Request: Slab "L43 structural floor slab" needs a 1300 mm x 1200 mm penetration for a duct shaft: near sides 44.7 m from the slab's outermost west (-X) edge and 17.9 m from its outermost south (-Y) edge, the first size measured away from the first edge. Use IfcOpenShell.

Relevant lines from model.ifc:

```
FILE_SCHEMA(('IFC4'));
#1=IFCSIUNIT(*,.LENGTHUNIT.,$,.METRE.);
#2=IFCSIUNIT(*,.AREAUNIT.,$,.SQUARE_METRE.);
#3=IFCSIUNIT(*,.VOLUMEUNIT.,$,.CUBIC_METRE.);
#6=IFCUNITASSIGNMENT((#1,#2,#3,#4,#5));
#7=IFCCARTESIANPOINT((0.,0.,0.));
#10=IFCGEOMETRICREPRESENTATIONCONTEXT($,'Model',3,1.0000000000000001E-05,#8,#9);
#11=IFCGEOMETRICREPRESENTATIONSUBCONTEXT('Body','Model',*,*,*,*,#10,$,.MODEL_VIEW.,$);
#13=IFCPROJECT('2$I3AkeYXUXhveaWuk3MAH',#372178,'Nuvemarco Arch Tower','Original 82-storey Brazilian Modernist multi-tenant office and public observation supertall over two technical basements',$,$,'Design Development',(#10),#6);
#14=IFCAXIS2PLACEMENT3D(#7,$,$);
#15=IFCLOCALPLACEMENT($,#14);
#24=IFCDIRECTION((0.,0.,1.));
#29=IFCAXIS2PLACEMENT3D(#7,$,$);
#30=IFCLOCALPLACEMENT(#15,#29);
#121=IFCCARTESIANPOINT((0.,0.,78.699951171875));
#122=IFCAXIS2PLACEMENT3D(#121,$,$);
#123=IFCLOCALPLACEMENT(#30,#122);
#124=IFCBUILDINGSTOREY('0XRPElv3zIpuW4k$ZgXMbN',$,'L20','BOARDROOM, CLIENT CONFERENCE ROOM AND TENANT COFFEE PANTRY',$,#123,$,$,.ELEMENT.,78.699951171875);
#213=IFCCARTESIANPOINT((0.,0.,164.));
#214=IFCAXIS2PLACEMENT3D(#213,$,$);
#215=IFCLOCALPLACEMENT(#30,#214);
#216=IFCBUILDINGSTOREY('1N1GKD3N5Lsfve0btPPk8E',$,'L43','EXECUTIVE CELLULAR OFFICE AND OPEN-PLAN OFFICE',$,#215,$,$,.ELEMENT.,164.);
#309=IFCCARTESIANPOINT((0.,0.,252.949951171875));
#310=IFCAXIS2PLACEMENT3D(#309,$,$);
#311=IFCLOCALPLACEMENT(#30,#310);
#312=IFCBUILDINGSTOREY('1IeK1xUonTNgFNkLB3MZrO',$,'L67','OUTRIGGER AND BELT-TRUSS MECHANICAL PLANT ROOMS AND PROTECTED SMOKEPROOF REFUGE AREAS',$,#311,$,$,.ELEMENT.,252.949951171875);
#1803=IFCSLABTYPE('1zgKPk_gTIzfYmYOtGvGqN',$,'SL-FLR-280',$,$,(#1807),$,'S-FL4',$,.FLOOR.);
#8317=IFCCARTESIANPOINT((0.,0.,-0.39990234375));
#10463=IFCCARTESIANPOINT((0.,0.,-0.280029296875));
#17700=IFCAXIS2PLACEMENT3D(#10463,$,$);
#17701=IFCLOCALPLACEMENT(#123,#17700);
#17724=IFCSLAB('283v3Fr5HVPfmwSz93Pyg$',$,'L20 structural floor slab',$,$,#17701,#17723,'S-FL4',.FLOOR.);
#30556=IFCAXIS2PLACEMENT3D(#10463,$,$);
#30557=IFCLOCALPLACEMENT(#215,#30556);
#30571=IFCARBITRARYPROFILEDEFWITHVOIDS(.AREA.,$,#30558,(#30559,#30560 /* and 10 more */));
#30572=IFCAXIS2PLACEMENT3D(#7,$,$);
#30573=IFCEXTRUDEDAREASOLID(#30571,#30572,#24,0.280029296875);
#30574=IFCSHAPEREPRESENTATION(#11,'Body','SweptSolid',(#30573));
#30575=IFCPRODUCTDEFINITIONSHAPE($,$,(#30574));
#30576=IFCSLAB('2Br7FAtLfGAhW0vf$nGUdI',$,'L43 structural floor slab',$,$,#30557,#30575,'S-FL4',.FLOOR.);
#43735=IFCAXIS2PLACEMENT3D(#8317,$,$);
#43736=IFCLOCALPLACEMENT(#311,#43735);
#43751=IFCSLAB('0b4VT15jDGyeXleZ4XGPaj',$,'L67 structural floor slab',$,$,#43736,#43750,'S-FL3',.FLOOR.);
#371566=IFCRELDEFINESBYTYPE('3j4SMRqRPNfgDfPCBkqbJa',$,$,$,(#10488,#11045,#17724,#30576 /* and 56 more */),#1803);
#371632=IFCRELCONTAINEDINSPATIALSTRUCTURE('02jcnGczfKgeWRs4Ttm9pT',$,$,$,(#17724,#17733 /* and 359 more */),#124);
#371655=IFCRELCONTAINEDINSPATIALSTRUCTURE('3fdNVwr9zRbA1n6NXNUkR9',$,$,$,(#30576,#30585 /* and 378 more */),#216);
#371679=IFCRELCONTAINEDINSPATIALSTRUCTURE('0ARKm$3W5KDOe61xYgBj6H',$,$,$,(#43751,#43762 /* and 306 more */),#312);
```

```python
import numpy as np
import ifcopenshell
import ifcopenshell.api.feature
import ifcopenshell.api.geometry
import ifcopenshell.api.root
import ifcopenshell.geom
import ifcopenshell.util.placement
import ifcopenshell.util.representation
import ifcopenshell.util.shape
import ifcopenshell.util.unit

model = ifcopenshell.open("model.ifc")
unit_scale = ifcopenshell.util.unit.calculate_unit_scale(model)
settings = ifcopenshell.geom.settings()


def volume(element):
    """Net volume in cubic metres, openings subtracted."""
    shape = ifcopenshell.geom.create_shape(settings, element)
    return ifcopenshell.util.shape.get_volume(shape.geometry)


slab = model.by_guid("2Br7FAtLfGAhW0vf$nGUdI")
before = volume(slab)

# Extent in the slab's own axes, in metres. The edges named are its -X and -Y sides.
slab_shape = ifcopenshell.geom.create_shape(settings, slab)
vertices = ifcopenshell.util.shape.get_vertices(slab_shape.geometry)
x_min, y_min, bottom = vertices.min(axis=0)
top = vertices[:, 2].max()

opening = ifcopenshell.api.root.create_entity(model, ifc_class="IfcOpeningElement", name="Duct shaft opening", predefined_type="OPENING")
context = ifcopenshell.util.representation.get_context(model, "Model", "Body", "MODEL_VIEW")
width, depth = 1.3, 1.2
outline = [(0.0, 0.0), (width, 0.0), (width, depth), (0.0, depth), (0.0, 0.0)]
# Overshoot both faces by 50 mm so the cut is clean.
shape = ifcopenshell.api.geometry.add_slab_representation(
    model, context=context, depth=top - bottom + 0.1, polyline=outline
)
ifcopenshell.api.geometry.assign_representation(model, product=opening, representation=shape)

matrix = ifcopenshell.util.placement.get_local_placement(slab.ObjectPlacement)
matrix[:, 3] = matrix @ np.append(np.array([x_min + 44.7, y_min + 17.9, bottom - 0.05]) / unit_scale, 1.0)
ifcopenshell.api.geometry.edit_object_placement(model, product=opening, matrix=matrix, is_si=False)
ifcopenshell.api.feature.add_feature(model, feature=opening, element=slab)

after = volume(slab)

print(f"slab volume {before:.3f} -> {after:.3f} m3")

model.write("model_v2.ifc")
```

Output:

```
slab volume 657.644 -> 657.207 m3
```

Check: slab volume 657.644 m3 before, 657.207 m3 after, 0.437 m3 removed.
